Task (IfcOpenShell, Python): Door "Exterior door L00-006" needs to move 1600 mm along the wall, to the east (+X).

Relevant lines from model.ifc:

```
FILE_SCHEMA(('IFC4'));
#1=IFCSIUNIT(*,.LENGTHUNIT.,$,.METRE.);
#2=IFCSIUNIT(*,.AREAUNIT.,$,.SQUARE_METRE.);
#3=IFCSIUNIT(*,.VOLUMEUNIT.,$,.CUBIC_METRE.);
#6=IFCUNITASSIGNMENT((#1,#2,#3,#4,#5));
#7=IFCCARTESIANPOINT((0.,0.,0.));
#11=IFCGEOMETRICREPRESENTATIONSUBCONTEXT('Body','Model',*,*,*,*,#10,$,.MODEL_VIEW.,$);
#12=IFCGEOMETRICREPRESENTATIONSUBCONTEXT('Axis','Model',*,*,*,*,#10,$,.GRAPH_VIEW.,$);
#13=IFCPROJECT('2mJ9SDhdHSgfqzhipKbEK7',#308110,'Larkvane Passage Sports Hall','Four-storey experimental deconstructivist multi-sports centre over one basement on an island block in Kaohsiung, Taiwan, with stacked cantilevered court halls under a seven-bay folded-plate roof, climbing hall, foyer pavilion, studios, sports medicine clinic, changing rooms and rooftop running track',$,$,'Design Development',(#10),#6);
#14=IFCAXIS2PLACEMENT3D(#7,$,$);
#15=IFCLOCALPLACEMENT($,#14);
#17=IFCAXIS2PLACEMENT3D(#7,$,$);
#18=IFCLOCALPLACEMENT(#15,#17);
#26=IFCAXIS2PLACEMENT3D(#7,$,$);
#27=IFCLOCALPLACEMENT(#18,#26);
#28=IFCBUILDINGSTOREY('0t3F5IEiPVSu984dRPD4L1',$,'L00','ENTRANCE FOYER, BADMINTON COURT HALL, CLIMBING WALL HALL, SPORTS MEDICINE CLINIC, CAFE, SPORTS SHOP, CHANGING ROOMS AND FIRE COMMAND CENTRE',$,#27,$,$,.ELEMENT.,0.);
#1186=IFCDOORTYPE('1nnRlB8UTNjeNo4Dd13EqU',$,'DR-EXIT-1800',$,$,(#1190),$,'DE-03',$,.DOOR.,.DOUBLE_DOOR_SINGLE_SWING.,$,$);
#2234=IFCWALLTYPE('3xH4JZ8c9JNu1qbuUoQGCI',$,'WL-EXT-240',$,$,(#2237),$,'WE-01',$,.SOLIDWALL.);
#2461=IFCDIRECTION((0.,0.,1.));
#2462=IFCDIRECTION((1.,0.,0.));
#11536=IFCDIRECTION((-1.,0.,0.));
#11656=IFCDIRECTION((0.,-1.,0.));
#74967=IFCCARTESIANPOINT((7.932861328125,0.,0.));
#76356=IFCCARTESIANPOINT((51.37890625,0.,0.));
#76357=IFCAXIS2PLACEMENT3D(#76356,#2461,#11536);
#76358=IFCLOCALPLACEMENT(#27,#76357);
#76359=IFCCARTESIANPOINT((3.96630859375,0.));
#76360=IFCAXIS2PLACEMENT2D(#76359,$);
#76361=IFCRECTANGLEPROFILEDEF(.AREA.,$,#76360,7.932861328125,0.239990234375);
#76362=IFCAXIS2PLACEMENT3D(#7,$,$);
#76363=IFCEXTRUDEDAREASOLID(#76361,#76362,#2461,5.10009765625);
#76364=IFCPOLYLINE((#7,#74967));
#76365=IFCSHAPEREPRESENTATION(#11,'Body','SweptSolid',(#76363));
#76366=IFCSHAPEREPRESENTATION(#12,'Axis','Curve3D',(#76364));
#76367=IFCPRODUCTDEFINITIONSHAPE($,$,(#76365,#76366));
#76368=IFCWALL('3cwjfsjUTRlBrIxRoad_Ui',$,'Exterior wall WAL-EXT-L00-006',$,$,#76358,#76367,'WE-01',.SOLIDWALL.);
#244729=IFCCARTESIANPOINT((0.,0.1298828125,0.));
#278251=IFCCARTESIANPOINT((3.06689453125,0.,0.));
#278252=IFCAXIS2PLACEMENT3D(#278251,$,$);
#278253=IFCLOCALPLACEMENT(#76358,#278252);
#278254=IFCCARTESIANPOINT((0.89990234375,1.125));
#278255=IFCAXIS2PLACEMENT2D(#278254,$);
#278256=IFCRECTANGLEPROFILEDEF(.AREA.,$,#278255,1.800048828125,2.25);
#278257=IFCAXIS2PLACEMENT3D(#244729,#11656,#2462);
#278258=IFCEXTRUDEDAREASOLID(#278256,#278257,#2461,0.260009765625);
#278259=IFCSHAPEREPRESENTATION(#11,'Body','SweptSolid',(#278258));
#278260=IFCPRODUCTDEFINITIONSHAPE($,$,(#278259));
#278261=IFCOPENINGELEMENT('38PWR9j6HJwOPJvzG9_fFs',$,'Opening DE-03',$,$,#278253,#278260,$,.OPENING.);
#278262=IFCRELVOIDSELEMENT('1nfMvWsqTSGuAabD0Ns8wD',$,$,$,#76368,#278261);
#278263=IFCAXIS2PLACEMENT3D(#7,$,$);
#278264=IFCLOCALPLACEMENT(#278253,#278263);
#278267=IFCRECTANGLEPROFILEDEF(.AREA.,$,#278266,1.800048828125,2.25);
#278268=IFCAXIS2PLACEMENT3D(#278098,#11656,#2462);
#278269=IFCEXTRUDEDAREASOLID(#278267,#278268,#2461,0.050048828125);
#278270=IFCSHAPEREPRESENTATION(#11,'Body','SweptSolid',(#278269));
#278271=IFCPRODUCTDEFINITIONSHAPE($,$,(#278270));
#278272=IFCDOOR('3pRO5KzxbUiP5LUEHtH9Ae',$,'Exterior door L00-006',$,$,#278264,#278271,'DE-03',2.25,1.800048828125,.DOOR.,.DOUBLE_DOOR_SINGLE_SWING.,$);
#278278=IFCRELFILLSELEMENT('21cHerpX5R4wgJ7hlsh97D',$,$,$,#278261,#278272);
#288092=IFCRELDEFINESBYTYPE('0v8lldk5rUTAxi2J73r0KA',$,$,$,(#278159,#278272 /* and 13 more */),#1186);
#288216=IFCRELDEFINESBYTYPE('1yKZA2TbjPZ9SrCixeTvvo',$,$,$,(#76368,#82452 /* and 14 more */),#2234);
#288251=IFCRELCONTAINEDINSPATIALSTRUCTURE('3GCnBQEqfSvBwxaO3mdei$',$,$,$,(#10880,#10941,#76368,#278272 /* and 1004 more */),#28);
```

```python
import ifcopenshell
import ifcopenshell.api.geometry
import ifcopenshell.util.placement
import ifcopenshell.util.unit

model = ifcopenshell.open("model.ifc")
unit_scale = ifcopenshell.util.unit.calculate_unit_scale(model)

door = model.by_guid("3pRO5KzxbUiP5LUEHtH9Ae")
opening = door.FillsVoids[0].RelatingOpeningElement
wall = opening.VoidsElements[0].RelatingBuildingElement

wall_matrix = ifcopenshell.util.placement.get_local_placement(wall.ObjectPlacement)
shift = wall_matrix[:3, 0] * -1.6 / unit_scale
before = ifcopenshell.util.placement.get_local_placement(door.ObjectPlacement)[:3, 3].copy()

# The door is placed relative to its opening, so it follows when the opening moves.
matrix = ifcopenshell.util.placement.get_local_placement(opening.ObjectPlacement)
matrix[:3, 3] += shift
ifcopenshell.api.geometry.edit_object_placement(
    model, product=opening, matrix=matrix, is_si=False, should_transform_children=True
)

after = ifcopenshell.util.placement.get_local_placement(door.ObjectPlacement)[:3, 3]
print("door moved by", (after - before).round(3) + 0.0)

model.write("model_updated.ifc")
```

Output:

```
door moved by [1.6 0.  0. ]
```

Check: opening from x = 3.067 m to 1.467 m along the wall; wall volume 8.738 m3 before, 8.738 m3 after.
